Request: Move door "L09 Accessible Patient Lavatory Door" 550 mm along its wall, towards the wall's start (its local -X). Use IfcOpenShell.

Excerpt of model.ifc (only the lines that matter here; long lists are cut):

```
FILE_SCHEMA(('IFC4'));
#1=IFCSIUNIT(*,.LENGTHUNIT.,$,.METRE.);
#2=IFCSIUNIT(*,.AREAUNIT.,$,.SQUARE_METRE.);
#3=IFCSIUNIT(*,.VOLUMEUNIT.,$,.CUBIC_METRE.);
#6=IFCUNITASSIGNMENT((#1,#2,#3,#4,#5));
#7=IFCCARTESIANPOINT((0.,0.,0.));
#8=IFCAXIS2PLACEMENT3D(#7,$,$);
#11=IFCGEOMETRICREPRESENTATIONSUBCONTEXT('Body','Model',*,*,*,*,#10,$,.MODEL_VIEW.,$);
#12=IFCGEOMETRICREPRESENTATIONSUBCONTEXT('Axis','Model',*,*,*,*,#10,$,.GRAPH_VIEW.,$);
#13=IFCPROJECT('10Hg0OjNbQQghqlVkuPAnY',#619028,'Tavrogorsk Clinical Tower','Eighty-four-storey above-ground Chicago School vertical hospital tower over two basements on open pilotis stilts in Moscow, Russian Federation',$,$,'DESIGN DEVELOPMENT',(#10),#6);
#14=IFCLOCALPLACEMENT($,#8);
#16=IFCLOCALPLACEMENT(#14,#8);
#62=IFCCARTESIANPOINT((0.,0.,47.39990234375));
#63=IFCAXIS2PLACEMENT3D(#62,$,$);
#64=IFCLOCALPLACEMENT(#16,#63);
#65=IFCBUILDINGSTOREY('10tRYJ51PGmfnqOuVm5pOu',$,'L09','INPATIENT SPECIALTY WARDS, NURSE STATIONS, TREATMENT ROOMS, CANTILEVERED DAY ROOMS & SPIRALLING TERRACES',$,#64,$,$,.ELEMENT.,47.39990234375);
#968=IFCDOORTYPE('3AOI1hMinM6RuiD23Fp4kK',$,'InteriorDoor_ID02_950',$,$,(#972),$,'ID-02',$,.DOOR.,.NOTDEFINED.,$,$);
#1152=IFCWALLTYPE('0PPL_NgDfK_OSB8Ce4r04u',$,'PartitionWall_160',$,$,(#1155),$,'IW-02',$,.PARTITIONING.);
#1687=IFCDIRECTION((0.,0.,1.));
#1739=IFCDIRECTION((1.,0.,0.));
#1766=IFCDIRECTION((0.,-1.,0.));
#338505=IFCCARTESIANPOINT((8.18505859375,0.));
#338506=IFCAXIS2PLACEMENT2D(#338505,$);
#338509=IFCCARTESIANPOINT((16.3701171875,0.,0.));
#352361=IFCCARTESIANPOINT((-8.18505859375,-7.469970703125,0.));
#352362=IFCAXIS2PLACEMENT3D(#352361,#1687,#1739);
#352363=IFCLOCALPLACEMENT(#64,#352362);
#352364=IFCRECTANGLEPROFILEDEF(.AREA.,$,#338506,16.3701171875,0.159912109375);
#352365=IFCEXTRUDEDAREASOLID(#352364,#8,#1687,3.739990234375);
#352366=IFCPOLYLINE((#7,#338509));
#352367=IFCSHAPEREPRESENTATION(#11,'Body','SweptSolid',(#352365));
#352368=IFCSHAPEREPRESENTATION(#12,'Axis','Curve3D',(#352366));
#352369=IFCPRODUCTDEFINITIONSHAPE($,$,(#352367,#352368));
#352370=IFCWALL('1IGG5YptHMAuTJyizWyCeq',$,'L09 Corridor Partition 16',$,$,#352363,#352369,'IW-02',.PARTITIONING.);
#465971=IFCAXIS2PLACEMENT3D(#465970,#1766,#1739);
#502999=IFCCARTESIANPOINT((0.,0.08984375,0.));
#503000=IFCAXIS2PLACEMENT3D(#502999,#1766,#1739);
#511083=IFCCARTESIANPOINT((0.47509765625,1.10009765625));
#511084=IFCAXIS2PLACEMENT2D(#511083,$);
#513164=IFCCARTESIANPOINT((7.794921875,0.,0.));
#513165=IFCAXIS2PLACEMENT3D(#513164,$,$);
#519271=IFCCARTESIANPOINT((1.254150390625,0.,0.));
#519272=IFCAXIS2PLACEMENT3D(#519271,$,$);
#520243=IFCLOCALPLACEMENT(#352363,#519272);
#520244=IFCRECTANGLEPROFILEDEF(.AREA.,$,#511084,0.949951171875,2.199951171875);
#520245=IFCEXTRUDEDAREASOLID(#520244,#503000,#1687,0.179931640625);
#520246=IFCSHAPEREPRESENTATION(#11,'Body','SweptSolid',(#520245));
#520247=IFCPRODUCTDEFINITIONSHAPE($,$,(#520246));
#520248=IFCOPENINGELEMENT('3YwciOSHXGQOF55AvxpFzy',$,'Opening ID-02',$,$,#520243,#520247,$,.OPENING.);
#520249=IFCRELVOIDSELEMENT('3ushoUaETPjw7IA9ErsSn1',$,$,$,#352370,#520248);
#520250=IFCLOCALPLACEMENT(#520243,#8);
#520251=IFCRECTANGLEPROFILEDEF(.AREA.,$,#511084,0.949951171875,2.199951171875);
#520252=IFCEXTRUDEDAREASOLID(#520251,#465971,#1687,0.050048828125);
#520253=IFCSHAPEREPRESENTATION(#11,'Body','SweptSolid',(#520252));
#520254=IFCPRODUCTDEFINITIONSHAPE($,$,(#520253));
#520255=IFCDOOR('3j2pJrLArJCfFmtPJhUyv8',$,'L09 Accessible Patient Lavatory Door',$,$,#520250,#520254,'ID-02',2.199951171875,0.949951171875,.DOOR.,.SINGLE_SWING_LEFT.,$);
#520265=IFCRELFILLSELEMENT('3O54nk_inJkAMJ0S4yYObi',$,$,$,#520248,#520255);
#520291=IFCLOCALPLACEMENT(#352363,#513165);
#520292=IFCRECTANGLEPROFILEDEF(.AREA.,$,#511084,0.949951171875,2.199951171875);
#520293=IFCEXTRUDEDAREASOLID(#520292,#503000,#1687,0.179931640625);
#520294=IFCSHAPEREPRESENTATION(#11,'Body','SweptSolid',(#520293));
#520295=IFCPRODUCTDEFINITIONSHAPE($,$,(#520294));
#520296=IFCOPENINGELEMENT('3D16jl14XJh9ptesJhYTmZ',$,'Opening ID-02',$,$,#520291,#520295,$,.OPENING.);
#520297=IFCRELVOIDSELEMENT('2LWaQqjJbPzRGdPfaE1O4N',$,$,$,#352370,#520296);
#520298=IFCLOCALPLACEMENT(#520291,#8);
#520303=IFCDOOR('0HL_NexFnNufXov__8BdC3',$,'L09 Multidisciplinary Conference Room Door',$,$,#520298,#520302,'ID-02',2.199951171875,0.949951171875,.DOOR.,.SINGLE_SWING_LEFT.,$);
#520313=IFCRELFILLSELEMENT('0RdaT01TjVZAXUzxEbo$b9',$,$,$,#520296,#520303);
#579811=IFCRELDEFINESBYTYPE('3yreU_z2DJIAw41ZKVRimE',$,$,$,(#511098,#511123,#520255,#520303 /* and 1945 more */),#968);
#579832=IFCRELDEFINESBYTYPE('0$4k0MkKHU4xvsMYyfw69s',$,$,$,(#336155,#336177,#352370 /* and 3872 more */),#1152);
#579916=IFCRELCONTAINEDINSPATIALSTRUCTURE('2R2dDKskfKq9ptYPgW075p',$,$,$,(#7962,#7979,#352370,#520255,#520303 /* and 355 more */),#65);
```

```python
import ifcopenshell
import ifcopenshell.api.geometry
import ifcopenshell.util.placement
import ifcopenshell.util.unit

model = ifcopenshell.open("model.ifc")
unit_scale = ifcopenshell.util.unit.calculate_unit_scale(model)

door = model.by_guid("3j2pJrLArJCfFmtPJhUyv8")
opening = door.FillsVoids[0].RelatingOpeningElement
wall = opening.VoidsElements[0].RelatingBuildingElement

wall_matrix = ifcopenshell.util.placement.get_local_placement(wall.ObjectPlacement)
shift = wall_matrix[:3, 0] * -0.55 / unit_scale
before = ifcopenshell.util.placement.get_local_placement(door.ObjectPlacement)[:3, 3].copy()

# The door is placed relative to its opening, so it follows when the opening moves.
matrix = ifcopenshell.util.placement.get_local_placement(opening.ObjectPlacement)
matrix[:3, 3] += shift
ifcopenshell.api.geometry.edit_object_placement(
    model, product=opening, matrix=matrix, is_si=False, should_transform_children=True
)

after = ifcopenshell.util.placement.get_local_placement(door.ObjectPlacement)[:3, 3]
print("door moved by", (after - before).round(3) + 0.0)

model.write("model_updated.ifc")
```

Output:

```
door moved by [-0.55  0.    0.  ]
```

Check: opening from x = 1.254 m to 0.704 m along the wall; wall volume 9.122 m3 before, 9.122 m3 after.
